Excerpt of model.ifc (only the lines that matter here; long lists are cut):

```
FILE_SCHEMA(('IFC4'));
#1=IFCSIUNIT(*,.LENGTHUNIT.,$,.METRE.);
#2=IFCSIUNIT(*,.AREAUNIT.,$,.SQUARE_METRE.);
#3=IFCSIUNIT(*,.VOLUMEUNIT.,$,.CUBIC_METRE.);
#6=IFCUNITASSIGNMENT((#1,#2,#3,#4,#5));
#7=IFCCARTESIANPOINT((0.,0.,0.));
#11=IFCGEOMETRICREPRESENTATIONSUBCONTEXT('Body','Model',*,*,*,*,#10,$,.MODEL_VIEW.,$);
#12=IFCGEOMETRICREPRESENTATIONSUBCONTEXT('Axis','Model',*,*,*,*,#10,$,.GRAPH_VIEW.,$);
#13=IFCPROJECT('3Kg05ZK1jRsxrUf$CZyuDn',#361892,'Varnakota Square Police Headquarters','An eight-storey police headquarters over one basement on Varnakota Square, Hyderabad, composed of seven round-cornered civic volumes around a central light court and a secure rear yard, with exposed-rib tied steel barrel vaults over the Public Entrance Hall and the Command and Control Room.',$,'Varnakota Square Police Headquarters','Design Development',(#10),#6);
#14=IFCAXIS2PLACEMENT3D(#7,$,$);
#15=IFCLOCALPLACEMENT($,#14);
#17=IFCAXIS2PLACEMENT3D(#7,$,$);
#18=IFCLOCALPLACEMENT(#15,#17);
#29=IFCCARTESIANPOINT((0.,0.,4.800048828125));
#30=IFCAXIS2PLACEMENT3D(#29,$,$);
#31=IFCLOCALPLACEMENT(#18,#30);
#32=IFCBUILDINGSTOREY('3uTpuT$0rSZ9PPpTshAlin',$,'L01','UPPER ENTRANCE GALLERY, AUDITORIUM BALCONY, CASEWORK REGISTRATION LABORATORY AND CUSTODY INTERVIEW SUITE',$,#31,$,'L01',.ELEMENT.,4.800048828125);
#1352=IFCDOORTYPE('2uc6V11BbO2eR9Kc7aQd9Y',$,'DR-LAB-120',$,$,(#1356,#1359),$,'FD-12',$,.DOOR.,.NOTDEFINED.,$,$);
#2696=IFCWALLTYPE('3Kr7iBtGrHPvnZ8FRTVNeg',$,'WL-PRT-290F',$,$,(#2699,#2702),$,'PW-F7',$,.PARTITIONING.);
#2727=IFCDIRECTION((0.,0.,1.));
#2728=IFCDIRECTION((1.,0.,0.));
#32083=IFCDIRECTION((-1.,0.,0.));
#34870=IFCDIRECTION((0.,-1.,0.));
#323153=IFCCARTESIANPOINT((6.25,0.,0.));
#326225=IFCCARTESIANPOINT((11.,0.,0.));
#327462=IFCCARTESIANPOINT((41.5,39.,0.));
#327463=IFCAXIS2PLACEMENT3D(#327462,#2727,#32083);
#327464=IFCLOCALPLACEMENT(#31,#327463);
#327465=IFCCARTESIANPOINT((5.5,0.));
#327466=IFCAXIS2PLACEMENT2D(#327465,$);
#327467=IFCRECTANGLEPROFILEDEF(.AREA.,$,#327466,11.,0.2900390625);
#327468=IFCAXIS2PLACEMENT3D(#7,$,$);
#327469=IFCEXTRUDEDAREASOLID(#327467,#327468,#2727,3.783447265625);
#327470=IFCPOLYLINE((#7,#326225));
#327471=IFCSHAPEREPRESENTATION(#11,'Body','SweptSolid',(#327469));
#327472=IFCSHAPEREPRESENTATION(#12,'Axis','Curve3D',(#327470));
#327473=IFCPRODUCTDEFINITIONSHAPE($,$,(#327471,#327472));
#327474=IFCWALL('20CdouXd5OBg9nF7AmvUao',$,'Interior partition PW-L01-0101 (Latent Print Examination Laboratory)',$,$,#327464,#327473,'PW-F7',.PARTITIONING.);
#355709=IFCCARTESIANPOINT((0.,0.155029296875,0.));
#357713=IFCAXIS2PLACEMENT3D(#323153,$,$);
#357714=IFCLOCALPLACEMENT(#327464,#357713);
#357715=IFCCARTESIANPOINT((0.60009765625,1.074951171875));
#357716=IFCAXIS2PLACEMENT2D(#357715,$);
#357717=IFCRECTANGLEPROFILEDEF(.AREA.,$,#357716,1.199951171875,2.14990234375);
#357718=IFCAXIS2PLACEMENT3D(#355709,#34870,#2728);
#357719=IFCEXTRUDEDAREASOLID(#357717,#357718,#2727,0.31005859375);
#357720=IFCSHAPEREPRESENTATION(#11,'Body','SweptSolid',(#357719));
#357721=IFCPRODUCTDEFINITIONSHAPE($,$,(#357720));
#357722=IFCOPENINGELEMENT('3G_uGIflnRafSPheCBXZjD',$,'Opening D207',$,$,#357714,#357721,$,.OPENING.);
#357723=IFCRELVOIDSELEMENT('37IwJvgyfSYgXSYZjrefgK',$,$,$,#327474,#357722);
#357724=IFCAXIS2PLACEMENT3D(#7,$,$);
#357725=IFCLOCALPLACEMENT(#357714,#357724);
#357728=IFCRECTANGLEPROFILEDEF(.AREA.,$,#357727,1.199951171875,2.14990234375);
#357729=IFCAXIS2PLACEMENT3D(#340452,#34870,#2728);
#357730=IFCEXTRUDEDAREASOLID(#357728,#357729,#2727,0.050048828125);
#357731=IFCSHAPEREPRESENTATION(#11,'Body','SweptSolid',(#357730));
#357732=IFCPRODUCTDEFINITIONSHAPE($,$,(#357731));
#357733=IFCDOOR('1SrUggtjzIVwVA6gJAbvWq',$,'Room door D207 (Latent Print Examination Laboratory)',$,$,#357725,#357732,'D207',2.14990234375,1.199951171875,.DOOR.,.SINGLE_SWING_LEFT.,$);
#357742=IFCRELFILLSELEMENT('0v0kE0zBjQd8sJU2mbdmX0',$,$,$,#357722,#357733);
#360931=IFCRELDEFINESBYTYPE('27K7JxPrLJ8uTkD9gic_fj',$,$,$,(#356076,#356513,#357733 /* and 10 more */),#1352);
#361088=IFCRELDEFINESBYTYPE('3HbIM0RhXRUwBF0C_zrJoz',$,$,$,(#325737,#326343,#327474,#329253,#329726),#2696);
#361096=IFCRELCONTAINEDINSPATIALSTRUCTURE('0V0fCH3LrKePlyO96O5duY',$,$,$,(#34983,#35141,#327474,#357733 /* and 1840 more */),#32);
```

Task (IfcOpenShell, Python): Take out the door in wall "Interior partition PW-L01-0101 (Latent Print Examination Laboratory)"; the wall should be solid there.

```python
import ifcopenshell
import ifcopenshell.api.feature
import ifcopenshell.api.root
import ifcopenshell.geom
import ifcopenshell.util.shape

model = ifcopenshell.open("model.ifc")
settings = ifcopenshell.geom.settings()


def volume(element):
    """Net volume in cubic metres, openings subtracted."""
    shape = ifcopenshell.geom.create_shape(settings, element)
    return ifcopenshell.util.shape.get_volume(shape.geometry)


door = model.by_id(357733)
opening = door.FillsVoids[0].RelatingOpeningElement
wall = opening.VoidsElements[0].RelatingBuildingElement
before = volume(wall)

ifcopenshell.api.root.remove_product(model, product=door)
ifcopenshell.api.feature.remove_feature(model, feature=opening)

after = volume(wall)

print(f"wall volume {before:.3f} -> {after:.3f} m3")

model.write("model_rev.ifc")
```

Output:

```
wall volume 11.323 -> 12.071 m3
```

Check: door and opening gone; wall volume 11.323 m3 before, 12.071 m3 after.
